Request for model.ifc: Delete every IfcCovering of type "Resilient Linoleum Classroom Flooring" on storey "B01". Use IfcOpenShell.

First a look at what the model holds.

```python
import ifcopenshell
import ifcopenshell.util.element

model = ifcopenshell.open("model.ifc")
print(model.schema)
storey = next(s for s in model.by_type("IfcBuildingStorey") if s.Name == "B01")
coverings = [e for e in ifcopenshell.util.element.get_decomposition(storey) if e.is_a("IfcCovering")]
seen = {}
for e in coverings:
    element_type = ifcopenshell.util.element.get_type(e)
    name = element_type.Name if element_type not in (None, e) else None
    seen[name] = seen.get(name, 0) + 1
for name, count in sorted(seen.items(), key=str):
    print(count, "x", name)
```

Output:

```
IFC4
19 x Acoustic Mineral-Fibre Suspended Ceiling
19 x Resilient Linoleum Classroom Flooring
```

```python
import ifcopenshell
import ifcopenshell.api.root
import ifcopenshell.util.element

model = ifcopenshell.open("model.ifc")

storey = next(s for s in model.by_type("IfcBuildingStorey") if s.Name == "B01")
coverings = [e for e in ifcopenshell.util.element.get_decomposition(storey) if e.is_a("IfcCovering")]
targets = [e for e in coverings if (t := ifcopenshell.util.element.get_type(e)) not in (None, e) and t.Name == "Resilient Linoleum Classroom Flooring"]

for e in targets:
    ifcopenshell.api.root.remove_product(model, product=e)
print(len(targets), "removed")

model.write("model_edited.ifc")
```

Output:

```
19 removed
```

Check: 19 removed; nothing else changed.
